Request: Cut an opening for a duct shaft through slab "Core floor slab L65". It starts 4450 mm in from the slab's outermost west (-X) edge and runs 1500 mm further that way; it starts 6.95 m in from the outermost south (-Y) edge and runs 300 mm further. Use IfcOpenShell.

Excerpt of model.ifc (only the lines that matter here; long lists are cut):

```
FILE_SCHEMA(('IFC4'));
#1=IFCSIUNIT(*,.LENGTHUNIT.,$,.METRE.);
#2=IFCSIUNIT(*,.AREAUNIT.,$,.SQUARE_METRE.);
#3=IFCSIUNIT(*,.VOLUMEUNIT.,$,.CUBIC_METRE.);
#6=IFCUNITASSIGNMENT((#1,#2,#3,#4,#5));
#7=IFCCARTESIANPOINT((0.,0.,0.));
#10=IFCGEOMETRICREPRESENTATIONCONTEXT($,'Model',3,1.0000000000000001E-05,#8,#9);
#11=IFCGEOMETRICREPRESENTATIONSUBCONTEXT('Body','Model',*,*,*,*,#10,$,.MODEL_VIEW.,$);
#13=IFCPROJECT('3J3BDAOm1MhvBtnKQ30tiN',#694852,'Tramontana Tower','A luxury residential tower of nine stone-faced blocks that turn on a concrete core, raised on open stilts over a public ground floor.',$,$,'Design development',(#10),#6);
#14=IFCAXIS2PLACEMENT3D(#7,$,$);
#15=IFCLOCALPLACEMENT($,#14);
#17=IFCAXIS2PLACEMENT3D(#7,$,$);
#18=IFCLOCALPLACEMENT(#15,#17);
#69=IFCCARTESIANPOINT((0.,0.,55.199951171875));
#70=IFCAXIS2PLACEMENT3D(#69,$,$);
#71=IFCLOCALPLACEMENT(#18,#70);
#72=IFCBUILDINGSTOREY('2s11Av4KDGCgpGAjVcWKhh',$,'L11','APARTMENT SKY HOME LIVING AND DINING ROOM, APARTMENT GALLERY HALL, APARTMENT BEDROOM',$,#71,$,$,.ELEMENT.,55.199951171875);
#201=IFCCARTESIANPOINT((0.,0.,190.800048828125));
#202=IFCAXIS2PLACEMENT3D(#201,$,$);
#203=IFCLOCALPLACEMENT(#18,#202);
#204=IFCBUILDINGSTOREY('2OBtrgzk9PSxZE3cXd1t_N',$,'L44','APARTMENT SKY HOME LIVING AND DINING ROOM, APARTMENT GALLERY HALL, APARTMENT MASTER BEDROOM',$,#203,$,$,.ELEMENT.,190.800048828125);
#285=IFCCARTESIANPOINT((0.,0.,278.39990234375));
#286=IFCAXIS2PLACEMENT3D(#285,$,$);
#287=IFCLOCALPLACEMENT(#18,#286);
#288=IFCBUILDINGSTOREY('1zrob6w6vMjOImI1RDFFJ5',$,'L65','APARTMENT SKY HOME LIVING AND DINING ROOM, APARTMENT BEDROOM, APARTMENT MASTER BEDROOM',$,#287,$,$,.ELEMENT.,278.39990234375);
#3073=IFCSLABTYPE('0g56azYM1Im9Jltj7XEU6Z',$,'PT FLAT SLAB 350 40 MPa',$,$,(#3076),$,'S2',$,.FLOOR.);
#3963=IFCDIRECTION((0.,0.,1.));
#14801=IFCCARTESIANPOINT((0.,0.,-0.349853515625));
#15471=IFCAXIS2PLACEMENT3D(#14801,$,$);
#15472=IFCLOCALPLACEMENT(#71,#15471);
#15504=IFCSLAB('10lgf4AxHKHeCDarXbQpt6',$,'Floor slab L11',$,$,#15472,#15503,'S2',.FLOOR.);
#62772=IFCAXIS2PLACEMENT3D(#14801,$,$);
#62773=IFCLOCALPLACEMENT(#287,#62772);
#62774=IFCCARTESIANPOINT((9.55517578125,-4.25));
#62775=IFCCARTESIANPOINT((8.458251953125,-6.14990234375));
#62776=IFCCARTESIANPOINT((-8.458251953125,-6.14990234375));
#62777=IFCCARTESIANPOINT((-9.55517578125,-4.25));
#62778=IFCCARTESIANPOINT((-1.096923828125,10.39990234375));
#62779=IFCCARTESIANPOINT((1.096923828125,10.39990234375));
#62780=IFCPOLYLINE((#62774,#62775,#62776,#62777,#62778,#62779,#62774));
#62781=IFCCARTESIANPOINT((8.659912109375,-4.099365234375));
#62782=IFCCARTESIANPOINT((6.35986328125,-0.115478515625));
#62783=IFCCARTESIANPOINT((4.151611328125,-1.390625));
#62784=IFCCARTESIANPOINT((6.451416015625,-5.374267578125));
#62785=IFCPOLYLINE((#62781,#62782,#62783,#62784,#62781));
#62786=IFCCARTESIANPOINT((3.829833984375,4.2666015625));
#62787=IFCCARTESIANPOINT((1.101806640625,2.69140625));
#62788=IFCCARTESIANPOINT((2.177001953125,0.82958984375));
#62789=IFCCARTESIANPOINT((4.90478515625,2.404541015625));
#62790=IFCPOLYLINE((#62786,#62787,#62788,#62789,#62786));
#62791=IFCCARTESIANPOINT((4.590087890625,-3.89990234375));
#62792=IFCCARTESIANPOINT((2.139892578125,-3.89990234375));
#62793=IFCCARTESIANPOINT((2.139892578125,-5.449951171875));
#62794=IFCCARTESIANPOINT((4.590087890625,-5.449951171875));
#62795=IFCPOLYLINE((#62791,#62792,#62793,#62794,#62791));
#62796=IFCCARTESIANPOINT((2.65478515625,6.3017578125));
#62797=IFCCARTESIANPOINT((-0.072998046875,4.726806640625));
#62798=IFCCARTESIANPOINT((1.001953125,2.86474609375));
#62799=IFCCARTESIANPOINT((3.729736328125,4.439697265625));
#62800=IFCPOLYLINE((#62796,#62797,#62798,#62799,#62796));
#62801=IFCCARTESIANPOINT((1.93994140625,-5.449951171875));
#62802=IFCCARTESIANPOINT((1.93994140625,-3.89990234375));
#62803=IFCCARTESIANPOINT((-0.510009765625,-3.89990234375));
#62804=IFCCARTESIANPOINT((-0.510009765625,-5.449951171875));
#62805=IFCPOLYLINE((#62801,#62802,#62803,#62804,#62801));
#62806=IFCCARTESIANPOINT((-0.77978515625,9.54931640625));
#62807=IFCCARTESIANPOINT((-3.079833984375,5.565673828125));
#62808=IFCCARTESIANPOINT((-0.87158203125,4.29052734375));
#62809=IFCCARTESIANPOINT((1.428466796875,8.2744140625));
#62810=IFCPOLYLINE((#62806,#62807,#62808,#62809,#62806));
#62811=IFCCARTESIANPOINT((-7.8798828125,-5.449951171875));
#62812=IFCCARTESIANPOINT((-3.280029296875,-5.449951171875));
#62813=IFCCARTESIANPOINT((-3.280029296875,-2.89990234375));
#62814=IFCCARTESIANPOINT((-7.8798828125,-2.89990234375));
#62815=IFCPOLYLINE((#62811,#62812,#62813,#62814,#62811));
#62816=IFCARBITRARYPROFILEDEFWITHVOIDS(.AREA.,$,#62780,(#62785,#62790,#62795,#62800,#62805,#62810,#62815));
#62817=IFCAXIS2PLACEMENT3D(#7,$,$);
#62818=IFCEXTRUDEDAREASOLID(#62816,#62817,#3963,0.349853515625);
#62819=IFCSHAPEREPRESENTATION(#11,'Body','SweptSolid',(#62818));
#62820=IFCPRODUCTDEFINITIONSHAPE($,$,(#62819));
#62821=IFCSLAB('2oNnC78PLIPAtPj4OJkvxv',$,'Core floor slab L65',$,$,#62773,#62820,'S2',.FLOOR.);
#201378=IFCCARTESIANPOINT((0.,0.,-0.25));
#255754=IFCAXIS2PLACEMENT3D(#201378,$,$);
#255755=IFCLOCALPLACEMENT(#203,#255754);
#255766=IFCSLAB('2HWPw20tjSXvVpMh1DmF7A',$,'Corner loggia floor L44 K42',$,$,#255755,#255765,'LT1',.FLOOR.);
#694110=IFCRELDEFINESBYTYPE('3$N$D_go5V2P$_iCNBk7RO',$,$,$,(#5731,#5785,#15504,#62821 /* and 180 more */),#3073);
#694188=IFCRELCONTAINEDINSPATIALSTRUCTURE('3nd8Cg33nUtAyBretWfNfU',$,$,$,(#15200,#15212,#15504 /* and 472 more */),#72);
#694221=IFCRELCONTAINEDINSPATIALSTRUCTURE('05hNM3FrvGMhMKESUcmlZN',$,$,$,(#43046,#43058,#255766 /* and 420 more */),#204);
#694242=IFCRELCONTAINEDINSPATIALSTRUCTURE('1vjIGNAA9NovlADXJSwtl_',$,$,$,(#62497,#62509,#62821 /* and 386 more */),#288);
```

```python
import numpy as np
import ifcopenshell
import ifcopenshell.api.feature
import ifcopenshell.api.geometry
import ifcopenshell.api.root
import ifcopenshell.geom
import ifcopenshell.util.placement
import ifcopenshell.util.representation
import ifcopenshell.util.shape
import ifcopenshell.util.unit

model = ifcopenshell.open("model.ifc")
unit_scale = ifcopenshell.util.unit.calculate_unit_scale(model)
settings = ifcopenshell.geom.settings()


def volume(element):
    """Net volume in cubic metres, openings subtracted."""
    shape = ifcopenshell.geom.create_shape(settings, element)
    return ifcopenshell.util.shape.get_volume(shape.geometry)


slab = model.by_id(62821)
before = volume(slab)

# Extent in the slab's own axes, in metres. The edges named are its -X and -Y sides.
slab_shape = ifcopenshell.geom.create_shape(settings, slab)
vertices = ifcopenshell.util.shape.get_vertices(slab_shape.geometry)
x_min, y_min, bottom = vertices.min(axis=0)
top = vertices[:, 2].max()

opening = ifcopenshell.api.root.create_entity(model, ifc_class="IfcOpeningElement", name="Duct shaft opening", predefined_type="OPENING")
context = ifcopenshell.util.representation.get_context(model, "Model", "Body", "MODEL_VIEW")
width, depth = 1.5, 0.3
outline = [(0.0, 0.0), (width, 0.0), (width, depth), (0.0, depth), (0.0, 0.0)]
# Overshoot both faces by 50 mm so the cut is clean.
shape = ifcopenshell.api.geometry.add_slab_representation(
    model, context=context, depth=top - bottom + 0.1, polyline=outline
)
ifcopenshell.api.geometry.assign_representation(model, product=opening, representation=shape)

matrix = ifcopenshell.util.placement.get_local_placement(slab.ObjectPlacement)
matrix[:, 3] = matrix @ np.append(np.array([x_min + 4.45, y_min + 6.95, bottom - 0.05]) / unit_scale, 1.0)
ifcopenshell.api.geometry.edit_object_placement(model, product=opening, matrix=matrix, is_si=False)
ifcopenshell.api.feature.add_feature(model, feature=opening, element=slab)

after = volume(slab)

print(f"slab volume {before:.3f} -> {after:.3f} m3")

model.write("model_edited.ifc")
```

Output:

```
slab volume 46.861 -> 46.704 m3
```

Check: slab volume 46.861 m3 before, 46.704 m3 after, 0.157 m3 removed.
